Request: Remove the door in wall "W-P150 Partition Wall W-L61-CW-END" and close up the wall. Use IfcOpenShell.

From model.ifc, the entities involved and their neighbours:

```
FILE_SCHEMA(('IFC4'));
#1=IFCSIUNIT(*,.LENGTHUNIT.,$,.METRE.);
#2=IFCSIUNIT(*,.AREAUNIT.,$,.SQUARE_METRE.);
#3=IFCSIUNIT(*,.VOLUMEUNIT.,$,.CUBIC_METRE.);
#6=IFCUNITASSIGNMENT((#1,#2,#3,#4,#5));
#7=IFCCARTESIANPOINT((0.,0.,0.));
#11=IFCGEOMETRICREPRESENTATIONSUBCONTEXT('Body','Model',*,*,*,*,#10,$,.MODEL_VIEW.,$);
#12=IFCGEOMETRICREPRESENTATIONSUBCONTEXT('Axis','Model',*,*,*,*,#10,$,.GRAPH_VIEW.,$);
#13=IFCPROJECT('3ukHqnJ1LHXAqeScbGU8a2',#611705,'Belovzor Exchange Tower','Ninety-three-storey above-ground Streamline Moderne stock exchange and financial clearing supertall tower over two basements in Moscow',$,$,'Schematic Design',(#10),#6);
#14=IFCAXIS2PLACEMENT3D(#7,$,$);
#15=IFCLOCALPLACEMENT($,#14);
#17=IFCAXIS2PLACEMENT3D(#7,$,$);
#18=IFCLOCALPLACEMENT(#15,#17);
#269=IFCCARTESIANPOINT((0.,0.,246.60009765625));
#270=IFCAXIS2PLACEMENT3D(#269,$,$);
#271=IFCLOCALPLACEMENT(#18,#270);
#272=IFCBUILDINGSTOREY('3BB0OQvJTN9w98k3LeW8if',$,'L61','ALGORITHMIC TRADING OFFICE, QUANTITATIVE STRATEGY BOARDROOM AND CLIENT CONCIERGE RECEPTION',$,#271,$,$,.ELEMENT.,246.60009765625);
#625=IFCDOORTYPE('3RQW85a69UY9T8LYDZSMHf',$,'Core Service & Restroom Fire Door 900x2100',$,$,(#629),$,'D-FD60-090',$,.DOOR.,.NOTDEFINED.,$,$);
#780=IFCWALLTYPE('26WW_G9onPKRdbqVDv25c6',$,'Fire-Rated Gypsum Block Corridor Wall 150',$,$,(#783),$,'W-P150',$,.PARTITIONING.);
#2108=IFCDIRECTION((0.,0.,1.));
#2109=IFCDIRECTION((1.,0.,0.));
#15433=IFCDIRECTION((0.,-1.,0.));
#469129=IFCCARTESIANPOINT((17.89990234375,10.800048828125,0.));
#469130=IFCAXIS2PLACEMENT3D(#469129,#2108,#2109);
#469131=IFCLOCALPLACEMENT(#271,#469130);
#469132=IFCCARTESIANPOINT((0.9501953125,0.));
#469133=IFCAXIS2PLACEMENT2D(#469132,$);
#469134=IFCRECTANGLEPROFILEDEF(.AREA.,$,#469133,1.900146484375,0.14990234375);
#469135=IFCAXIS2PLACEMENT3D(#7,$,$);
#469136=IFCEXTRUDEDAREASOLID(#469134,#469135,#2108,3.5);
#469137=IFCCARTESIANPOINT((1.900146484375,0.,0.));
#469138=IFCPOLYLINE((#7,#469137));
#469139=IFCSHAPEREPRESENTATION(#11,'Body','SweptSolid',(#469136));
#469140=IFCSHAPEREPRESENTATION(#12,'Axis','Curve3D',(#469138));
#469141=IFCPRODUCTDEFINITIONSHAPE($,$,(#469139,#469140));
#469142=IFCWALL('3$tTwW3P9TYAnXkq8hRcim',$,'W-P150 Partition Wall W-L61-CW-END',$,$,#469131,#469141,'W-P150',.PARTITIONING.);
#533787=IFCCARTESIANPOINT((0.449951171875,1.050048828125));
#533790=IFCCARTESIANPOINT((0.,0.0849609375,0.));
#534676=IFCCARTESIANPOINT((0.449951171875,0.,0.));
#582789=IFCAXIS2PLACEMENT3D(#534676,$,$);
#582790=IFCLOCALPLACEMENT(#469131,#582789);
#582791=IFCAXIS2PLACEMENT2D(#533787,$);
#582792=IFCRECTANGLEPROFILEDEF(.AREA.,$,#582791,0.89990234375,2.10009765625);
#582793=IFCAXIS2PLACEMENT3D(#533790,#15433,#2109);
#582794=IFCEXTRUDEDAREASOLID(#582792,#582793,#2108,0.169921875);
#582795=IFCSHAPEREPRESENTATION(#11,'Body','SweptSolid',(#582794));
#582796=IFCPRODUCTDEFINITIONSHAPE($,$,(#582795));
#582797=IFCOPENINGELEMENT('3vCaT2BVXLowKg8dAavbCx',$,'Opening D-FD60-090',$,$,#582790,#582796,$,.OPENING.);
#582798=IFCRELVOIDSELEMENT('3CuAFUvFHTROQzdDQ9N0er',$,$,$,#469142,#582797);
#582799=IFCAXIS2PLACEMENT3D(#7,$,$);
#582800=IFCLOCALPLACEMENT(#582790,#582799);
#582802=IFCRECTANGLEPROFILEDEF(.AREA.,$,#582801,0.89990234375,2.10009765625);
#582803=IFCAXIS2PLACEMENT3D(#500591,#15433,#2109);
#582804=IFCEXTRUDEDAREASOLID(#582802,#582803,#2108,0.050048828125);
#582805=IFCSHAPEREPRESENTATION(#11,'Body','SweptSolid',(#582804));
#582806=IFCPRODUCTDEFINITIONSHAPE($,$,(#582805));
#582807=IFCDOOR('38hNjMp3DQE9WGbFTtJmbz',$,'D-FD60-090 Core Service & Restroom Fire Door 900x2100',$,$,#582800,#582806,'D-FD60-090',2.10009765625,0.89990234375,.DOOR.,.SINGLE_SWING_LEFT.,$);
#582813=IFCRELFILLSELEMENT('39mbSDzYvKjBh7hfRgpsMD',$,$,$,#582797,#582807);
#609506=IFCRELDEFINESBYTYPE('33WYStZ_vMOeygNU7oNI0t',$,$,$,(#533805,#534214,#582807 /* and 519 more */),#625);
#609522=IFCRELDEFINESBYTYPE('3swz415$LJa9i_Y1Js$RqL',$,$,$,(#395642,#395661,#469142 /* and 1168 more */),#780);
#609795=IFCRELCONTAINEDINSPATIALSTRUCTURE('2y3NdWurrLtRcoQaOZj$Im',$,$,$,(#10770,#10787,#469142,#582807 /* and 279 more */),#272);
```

```python
import ifcopenshell
import ifcopenshell.api.feature
import ifcopenshell.api.root
import ifcopenshell.geom
import ifcopenshell.util.shape

model = ifcopenshell.open("model.ifc")
settings = ifcopenshell.geom.settings()


def volume(element):
    """Net volume in cubic metres, openings subtracted."""
    shape = ifcopenshell.geom.create_shape(settings, element)
    return ifcopenshell.util.shape.get_volume(shape.geometry)


door = model.by_guid("38hNjMp3DQE9WGbFTtJmbz")
opening = door.FillsVoids[0].RelatingOpeningElement
wall = opening.VoidsElements[0].RelatingBuildingElement
before = volume(wall)

ifcopenshell.api.root.remove_product(model, product=door)
ifcopenshell.api.feature.remove_feature(model, feature=opening)

after = volume(wall)

print(f"wall volume {before:.3f} -> {after:.3f} m3")

model.write("model-out.ifc")
```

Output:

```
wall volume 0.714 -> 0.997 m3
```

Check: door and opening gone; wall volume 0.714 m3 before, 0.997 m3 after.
